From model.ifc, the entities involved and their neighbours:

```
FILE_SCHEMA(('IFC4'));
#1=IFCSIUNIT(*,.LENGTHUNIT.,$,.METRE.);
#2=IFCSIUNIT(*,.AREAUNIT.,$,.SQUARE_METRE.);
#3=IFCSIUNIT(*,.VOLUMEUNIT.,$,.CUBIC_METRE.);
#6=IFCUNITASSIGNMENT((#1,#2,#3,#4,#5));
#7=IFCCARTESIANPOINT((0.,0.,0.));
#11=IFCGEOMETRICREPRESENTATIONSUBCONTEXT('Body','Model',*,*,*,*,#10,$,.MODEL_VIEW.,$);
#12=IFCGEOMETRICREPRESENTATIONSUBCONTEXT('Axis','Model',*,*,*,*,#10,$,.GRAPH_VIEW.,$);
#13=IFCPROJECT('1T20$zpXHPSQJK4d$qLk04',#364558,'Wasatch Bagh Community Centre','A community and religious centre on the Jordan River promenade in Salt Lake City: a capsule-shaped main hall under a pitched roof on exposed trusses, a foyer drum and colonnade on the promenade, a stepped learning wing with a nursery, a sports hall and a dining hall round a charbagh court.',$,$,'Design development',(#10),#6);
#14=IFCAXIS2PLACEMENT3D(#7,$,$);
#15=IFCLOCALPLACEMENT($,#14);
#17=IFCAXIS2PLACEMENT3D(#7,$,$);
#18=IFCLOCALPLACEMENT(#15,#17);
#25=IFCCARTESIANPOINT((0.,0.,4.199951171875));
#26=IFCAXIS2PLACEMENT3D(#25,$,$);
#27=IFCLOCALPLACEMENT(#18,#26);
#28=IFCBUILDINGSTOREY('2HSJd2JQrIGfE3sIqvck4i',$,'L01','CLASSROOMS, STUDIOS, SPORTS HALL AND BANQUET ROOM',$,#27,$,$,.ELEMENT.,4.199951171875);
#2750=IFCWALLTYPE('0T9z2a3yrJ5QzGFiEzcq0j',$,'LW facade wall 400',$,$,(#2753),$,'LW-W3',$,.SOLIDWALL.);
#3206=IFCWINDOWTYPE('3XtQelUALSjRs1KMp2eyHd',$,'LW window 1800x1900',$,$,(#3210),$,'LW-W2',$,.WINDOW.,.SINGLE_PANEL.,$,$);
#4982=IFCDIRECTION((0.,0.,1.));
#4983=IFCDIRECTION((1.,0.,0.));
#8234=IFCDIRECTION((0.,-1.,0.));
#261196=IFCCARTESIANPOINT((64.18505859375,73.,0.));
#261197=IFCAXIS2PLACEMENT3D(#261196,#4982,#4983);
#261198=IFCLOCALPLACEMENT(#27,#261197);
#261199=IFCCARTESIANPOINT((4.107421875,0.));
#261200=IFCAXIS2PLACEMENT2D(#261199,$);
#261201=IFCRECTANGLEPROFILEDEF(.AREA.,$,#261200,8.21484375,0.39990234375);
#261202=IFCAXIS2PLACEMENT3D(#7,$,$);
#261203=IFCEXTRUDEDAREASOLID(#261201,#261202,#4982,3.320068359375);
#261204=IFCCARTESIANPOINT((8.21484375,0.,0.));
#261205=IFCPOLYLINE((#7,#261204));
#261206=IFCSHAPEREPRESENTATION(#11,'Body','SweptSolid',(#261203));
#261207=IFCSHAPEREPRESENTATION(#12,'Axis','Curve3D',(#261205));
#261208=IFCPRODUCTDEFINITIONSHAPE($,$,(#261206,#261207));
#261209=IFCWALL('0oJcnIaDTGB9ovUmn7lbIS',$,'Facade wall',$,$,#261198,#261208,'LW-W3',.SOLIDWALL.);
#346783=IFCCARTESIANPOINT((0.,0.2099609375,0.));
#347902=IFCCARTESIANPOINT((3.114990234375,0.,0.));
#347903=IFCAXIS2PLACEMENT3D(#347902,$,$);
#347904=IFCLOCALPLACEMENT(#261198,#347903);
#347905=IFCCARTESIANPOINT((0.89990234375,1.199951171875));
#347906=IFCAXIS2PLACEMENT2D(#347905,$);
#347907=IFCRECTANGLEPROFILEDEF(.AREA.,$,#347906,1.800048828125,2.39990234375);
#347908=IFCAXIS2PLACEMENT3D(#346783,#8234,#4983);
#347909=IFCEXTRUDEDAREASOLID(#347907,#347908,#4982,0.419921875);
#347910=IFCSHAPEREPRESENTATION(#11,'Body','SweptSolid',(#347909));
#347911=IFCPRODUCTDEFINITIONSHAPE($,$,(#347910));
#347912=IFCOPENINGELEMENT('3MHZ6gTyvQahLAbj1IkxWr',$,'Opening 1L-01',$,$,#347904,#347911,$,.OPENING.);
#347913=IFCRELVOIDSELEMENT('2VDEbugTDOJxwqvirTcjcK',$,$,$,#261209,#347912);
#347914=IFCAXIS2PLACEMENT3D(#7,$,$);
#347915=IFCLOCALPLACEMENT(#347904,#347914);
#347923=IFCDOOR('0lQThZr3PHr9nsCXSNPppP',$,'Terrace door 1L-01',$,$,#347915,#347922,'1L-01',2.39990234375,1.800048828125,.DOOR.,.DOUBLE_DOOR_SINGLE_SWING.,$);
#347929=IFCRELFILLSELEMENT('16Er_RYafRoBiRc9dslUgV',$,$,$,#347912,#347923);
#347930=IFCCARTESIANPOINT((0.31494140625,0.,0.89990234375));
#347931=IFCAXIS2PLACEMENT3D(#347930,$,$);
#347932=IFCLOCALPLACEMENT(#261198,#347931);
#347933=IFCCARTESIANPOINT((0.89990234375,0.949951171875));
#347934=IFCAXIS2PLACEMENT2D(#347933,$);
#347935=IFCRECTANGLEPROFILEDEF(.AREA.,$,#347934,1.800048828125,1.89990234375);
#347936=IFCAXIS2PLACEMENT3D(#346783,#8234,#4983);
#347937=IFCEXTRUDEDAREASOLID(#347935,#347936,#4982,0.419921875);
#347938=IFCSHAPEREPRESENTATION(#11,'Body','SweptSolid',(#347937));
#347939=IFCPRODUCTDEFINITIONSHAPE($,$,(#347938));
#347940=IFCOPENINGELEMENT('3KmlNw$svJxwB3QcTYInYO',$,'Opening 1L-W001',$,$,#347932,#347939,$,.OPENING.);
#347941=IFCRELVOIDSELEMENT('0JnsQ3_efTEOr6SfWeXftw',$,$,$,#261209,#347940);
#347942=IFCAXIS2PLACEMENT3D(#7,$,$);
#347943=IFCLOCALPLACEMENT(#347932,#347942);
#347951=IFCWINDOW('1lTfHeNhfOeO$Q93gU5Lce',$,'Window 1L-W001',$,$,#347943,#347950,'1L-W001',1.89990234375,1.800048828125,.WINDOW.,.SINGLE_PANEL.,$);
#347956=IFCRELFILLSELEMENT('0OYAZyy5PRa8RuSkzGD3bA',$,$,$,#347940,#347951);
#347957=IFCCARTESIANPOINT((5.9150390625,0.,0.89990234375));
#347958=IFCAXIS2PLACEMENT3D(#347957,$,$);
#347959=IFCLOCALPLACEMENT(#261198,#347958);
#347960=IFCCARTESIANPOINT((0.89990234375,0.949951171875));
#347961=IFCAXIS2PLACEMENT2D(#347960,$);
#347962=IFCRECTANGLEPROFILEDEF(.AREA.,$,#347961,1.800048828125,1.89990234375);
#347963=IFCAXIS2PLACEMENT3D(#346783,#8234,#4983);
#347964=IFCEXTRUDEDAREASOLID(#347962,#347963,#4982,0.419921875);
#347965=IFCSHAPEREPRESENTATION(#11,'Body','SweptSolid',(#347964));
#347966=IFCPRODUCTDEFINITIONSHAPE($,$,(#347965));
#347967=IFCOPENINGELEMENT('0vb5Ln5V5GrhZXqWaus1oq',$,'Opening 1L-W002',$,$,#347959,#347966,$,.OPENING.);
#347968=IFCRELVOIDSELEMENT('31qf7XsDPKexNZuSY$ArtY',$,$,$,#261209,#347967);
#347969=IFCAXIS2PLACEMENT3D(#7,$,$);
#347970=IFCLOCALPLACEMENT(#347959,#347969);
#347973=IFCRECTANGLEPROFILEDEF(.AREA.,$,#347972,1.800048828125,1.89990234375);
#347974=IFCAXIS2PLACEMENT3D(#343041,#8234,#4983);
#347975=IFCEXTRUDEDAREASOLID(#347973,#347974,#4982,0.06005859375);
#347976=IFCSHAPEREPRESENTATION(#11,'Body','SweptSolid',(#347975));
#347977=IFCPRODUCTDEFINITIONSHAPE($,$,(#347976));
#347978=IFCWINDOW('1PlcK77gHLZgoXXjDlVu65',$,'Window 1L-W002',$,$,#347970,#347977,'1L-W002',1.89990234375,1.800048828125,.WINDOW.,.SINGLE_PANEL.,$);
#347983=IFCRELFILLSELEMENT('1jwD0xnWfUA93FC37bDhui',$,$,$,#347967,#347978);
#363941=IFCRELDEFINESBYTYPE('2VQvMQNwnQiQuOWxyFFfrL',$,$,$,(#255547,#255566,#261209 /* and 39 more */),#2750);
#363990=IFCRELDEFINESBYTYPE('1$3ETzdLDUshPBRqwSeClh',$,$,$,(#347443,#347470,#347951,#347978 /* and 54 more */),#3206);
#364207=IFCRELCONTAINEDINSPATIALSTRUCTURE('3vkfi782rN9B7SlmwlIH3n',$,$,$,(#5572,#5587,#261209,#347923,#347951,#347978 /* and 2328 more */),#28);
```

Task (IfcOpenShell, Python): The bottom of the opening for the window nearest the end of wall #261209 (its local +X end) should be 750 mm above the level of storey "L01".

```python
import numpy as np
import ifcopenshell
import ifcopenshell.api.geometry
import ifcopenshell.geom
import ifcopenshell.util.element
import ifcopenshell.util.placement
import ifcopenshell.util.shape
import ifcopenshell.util.unit

model = ifcopenshell.open("model.ifc")
unit_scale = ifcopenshell.util.unit.calculate_unit_scale(model)

window = model.by_id(347978)
opening = window.FillsVoids[0].RelatingOpeningElement
storey = ifcopenshell.util.element.get_container(window, ifc_class="IfcBuildingStorey")
level = ifcopenshell.util.placement.get_local_placement(storey.ObjectPlacement)[2, 3]

# The opening's origin need not be at the sill, so measure its lowest point.
shape = ifcopenshell.geom.create_shape(ifcopenshell.geom.settings(), opening)
bottom = ifcopenshell.util.shape.get_shape_bottom_elevation(shape, shape.geometry) / unit_scale
dz = level + 0.75 / unit_scale - bottom

shift = np.array([0.0, 0.0, dz])
# The window is placed relative to its opening, so it follows when the opening moves.
matrix = ifcopenshell.util.placement.get_local_placement(opening.ObjectPlacement)
matrix[:3, 3] += shift
ifcopenshell.api.geometry.edit_object_placement(
    model, product=opening, matrix=matrix, is_si=False, should_transform_children=True
)

print(f"moved by {dz * unit_scale:+.3f} m")

model.write("model-out.ifc")
```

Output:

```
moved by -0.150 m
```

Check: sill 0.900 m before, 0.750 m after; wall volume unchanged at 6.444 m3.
